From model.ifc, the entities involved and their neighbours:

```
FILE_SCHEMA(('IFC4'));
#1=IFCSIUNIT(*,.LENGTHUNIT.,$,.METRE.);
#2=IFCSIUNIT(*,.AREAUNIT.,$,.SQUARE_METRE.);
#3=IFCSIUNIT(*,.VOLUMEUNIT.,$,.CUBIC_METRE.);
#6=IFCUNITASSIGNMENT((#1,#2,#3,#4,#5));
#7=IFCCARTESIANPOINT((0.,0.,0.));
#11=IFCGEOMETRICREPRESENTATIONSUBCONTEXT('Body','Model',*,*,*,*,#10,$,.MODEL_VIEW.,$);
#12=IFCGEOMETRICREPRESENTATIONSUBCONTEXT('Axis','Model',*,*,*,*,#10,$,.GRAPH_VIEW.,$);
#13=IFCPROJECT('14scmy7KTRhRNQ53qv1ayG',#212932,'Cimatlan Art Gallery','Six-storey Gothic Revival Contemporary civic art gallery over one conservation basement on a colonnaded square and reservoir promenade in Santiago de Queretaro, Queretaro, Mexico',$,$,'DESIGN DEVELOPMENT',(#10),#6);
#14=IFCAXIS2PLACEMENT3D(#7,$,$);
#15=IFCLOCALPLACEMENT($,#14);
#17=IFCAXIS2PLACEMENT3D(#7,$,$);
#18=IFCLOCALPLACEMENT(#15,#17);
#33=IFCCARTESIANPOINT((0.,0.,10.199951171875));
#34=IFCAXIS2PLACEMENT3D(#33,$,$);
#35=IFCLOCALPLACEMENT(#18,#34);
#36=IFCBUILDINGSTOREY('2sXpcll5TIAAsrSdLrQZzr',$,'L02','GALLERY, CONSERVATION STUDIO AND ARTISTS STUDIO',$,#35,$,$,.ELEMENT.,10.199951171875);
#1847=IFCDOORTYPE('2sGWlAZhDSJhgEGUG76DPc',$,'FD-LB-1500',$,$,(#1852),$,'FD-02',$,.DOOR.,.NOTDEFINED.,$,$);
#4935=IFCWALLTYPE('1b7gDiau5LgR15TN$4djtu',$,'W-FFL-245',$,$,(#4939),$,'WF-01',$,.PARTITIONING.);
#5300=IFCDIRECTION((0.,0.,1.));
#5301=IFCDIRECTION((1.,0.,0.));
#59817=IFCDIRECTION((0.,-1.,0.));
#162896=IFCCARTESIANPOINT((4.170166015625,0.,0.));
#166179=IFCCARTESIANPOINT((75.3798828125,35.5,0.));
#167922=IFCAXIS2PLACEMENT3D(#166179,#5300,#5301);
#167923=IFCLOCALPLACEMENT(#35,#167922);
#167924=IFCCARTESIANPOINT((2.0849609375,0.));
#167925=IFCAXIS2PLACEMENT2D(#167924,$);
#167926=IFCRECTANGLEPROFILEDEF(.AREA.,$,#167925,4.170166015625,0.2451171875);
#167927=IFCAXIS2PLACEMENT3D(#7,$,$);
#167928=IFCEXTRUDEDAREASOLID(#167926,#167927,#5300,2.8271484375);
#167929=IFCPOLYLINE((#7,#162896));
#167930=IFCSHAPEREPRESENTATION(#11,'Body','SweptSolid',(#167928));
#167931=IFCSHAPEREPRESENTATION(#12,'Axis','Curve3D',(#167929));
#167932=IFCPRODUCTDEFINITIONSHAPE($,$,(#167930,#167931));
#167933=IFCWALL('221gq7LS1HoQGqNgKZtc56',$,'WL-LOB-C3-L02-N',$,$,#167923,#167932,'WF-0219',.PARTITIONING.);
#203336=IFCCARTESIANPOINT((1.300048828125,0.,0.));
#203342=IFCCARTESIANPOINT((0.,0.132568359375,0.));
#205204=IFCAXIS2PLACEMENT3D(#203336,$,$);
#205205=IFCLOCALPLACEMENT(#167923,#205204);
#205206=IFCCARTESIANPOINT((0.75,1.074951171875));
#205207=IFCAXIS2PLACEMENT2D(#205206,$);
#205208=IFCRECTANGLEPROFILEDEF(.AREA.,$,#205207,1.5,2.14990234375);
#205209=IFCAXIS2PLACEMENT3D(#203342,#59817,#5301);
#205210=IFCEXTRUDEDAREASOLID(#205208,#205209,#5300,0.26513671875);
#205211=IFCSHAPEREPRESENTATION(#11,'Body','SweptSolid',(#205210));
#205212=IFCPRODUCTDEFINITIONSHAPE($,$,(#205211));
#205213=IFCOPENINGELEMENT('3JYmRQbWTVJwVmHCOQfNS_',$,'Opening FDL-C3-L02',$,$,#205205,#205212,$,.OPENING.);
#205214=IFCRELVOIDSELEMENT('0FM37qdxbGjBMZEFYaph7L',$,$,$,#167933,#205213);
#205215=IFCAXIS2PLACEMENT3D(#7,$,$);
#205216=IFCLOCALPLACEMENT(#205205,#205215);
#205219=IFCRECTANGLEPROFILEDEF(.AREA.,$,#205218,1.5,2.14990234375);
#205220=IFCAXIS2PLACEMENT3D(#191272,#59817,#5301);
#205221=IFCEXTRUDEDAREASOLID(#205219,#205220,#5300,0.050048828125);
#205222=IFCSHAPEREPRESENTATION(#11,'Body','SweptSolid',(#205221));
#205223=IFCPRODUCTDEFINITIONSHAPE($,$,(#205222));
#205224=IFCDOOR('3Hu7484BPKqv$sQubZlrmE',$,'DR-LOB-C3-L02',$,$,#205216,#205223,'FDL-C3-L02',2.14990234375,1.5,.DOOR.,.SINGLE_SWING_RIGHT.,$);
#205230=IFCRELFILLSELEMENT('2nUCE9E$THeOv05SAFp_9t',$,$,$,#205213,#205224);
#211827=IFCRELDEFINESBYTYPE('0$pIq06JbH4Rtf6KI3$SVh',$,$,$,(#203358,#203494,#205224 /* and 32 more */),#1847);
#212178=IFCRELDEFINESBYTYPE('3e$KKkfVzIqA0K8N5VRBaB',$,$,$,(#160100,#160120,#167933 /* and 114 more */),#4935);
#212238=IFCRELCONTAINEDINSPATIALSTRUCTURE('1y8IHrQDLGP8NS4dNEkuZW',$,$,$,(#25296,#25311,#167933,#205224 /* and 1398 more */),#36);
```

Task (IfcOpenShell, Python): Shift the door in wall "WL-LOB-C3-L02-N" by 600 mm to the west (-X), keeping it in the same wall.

```python
import ifcopenshell
import ifcopenshell.api.geometry
import ifcopenshell.util.placement

model = ifcopenshell.open("model.ifc")

door = model.by_guid("3Hu7484BPKqv$sQubZlrmE")
opening = door.FillsVoids[0].RelatingOpeningElement
wall = opening.VoidsElements[0].RelatingBuildingElement

wall_matrix = ifcopenshell.util.placement.get_local_placement(wall.ObjectPlacement)
shift = wall_matrix[:3, 0] * -0.6
before = ifcopenshell.util.placement.get_local_placement(door.ObjectPlacement)[:3, 3].copy()

# The door is placed relative to its opening, so it follows when the opening moves.
matrix = ifcopenshell.util.placement.get_local_placement(opening.ObjectPlacement)
matrix[:3, 3] += shift
ifcopenshell.api.geometry.edit_object_placement(
    model, product=opening, matrix=matrix, is_si=False, should_transform_children=True
)

after = ifcopenshell.util.placement.get_local_placement(door.ObjectPlacement)[:3, 3]
print("door moved by", (after - before).round(3) + 0.0)

model.write("model_rev.ifc")
```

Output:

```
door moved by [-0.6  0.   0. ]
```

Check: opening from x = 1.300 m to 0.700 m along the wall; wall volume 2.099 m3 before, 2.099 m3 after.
